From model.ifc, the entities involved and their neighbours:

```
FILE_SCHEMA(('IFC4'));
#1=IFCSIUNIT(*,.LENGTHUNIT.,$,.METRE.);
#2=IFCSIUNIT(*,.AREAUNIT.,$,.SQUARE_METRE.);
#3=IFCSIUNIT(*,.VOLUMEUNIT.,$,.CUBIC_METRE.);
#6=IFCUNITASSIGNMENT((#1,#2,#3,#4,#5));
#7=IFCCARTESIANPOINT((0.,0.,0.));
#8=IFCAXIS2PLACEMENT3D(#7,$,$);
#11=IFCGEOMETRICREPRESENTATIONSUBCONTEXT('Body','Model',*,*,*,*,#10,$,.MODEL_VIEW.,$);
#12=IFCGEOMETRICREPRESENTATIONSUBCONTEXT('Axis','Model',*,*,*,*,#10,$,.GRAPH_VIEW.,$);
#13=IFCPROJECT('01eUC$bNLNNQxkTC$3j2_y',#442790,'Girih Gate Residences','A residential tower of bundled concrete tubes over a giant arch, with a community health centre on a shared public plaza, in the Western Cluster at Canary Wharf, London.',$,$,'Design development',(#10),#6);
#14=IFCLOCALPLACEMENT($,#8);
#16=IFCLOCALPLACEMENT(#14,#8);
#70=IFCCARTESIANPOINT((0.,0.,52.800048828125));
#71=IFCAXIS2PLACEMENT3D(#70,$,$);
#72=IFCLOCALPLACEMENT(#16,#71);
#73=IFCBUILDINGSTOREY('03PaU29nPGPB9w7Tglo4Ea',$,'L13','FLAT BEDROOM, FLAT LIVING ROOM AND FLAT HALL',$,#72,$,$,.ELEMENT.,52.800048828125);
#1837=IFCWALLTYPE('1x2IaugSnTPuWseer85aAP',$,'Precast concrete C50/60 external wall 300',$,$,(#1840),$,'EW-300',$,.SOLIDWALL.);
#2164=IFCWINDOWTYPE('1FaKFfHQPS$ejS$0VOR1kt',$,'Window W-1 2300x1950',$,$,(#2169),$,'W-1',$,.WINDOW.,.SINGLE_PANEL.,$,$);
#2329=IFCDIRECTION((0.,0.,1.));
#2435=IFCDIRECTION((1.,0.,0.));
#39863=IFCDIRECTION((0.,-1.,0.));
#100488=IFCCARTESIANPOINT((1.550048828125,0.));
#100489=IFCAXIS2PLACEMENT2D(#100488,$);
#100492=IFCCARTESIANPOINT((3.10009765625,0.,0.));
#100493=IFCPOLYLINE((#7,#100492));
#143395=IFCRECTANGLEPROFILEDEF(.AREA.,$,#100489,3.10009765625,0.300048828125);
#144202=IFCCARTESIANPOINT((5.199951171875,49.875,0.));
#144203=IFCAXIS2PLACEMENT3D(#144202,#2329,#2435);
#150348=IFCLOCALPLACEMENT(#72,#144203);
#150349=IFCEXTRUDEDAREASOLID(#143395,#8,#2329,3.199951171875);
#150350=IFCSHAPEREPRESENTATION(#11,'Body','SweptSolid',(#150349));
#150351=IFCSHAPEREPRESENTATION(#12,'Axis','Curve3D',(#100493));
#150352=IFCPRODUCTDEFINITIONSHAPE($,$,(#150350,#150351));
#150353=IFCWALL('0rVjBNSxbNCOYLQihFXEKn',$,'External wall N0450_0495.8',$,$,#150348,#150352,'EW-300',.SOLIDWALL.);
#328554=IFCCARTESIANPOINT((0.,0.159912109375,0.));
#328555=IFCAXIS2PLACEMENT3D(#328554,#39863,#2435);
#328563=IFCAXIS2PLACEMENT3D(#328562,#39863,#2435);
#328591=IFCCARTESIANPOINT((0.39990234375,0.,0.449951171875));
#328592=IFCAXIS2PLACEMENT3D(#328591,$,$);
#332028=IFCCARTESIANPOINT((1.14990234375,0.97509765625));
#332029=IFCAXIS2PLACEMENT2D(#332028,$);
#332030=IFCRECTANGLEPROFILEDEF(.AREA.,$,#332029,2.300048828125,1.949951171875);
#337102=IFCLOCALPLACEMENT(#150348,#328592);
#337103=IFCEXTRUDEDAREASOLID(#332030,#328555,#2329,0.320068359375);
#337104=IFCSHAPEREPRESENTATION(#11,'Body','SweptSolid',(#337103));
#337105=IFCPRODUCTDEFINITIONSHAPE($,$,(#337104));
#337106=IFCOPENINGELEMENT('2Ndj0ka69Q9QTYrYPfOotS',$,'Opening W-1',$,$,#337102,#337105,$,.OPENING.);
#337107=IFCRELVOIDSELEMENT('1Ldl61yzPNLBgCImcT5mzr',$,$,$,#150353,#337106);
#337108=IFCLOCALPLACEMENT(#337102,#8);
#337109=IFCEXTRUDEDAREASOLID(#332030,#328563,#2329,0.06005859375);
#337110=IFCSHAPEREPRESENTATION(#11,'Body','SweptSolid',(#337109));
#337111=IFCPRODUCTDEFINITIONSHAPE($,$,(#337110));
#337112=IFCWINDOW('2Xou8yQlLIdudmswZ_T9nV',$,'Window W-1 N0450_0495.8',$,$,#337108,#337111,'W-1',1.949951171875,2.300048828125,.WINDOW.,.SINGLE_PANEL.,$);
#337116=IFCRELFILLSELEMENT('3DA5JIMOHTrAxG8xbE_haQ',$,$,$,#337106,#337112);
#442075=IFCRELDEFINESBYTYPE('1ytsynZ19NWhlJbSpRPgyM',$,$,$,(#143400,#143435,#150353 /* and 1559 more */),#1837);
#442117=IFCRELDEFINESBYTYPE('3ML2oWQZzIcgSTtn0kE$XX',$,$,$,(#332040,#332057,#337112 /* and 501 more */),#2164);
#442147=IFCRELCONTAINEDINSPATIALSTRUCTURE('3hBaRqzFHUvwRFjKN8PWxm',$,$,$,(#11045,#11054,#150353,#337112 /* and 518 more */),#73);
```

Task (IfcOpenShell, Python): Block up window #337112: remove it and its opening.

```python
import ifcopenshell
import ifcopenshell.api.feature
import ifcopenshell.api.root
import ifcopenshell.geom
import ifcopenshell.util.shape

model = ifcopenshell.open("model.ifc")
settings = ifcopenshell.geom.settings()


def volume(element):
    """Net volume in cubic metres, openings subtracted."""
    shape = ifcopenshell.geom.create_shape(settings, element)
    return ifcopenshell.util.shape.get_volume(shape.geometry)


window = model.by_guid("2Xou8yQlLIdudmswZ_T9nV")
opening = window.FillsVoids[0].RelatingOpeningElement
wall = opening.VoidsElements[0].RelatingBuildingElement
before = volume(wall)

ifcopenshell.api.root.remove_product(model, product=window)
ifcopenshell.api.feature.remove_feature(model, feature=opening)

after = volume(wall)

print(f"wall volume {before:.3f} -> {after:.3f} m3")

model.write("model_v2.ifc")
```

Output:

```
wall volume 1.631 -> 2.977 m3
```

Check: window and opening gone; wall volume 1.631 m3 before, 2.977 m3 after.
